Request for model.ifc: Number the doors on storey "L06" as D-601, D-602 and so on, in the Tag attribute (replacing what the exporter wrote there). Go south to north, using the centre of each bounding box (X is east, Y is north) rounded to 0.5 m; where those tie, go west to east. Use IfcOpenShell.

First a look at what the model holds.

```python
import ifcopenshell
import ifcopenshell.util.element
import ifcopenshell.util.placement

model = ifcopenshell.open("model.ifc")
print(model.schema)
storey = next(s for s in model.by_type("IfcBuildingStorey") if s.Name == "L06")
doors = [e for e in ifcopenshell.util.element.get_decomposition(storey) if e.is_a("IfcDoor")]
for e in sorted(doors, key=lambda e: e.id()):
    origin = ifcopenshell.util.placement.get_local_placement(e.ObjectPlacement)[:3, 3]
    print(e.id(), e.Tag, e.Name, origin.round(2) + 0.0, sep=" | ")
```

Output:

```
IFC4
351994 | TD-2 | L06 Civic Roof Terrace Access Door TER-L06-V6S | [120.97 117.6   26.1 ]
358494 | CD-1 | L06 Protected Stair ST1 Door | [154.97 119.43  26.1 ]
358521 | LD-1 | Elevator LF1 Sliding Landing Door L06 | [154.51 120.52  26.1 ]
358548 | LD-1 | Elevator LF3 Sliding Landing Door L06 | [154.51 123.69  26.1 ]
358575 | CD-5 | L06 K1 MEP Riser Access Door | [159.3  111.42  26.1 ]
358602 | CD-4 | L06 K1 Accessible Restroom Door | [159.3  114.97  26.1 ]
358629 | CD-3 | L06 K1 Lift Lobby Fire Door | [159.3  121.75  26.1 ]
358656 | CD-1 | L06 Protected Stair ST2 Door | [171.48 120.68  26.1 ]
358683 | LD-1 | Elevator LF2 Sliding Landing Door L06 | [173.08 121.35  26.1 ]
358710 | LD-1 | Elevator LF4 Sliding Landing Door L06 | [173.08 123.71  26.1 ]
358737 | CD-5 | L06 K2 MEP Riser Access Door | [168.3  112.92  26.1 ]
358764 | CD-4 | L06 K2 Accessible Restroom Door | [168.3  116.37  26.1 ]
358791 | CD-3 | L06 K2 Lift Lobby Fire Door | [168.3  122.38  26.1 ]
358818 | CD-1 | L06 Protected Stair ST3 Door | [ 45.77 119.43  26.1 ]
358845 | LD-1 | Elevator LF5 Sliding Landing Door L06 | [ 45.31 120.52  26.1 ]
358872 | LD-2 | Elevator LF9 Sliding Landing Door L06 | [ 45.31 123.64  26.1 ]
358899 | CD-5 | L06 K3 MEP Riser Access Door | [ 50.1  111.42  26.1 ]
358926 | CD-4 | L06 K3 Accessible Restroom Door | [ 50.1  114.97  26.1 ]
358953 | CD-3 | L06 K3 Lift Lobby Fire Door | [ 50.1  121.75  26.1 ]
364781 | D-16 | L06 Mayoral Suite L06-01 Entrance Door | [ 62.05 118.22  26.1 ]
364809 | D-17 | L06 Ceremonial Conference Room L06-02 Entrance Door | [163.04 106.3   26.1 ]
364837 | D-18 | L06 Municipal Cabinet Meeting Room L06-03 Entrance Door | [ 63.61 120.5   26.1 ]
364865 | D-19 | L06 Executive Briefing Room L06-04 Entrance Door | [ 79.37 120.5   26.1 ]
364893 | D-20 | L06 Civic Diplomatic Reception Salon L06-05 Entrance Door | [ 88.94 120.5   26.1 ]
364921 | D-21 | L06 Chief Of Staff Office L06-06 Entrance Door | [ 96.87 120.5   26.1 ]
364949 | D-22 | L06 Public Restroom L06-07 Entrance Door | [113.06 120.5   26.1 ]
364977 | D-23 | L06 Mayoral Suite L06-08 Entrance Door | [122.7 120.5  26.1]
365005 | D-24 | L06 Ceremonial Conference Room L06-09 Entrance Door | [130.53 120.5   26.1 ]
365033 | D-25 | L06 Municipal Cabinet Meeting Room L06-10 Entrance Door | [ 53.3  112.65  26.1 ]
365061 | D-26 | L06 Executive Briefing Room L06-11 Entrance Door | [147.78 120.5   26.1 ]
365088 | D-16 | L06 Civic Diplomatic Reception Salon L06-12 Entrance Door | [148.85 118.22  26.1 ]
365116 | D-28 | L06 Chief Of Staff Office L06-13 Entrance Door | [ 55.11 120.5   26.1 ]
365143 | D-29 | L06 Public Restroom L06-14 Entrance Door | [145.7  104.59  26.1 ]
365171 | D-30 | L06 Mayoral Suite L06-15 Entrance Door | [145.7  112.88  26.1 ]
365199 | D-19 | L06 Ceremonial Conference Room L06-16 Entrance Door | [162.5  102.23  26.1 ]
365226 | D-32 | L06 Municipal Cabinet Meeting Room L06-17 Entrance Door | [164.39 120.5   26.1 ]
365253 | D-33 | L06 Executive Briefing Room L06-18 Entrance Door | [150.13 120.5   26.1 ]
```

```python
import ifcopenshell
import ifcopenshell.geom
import ifcopenshell.util.element
import ifcopenshell.util.shape

model = ifcopenshell.open("model.ifc")
settings = ifcopenshell.geom.settings()
settings.set("use-world-coords", True)


def centre(element):
    shape = ifcopenshell.geom.create_shape(settings, element)
    return ifcopenshell.util.shape.get_bbox_centroid(shape.geometry)


storey = next(s for s in model.by_type("IfcBuildingStorey") if s.Name == "L06")
doors = [e for e in ifcopenshell.util.element.get_decomposition(storey) if e.is_a("IfcDoor")]

# Insertion points can sit at a corner or the storey origin, so sort by the geometry (in metres).
centres = {e: centre(e) for e in doors}
doors.sort(key=lambda e: (round(centres[e][1] / 0.5), centres[e][0]))

for i, e in enumerate(doors, start=1):
    number = f"D-6{i:02d}"
    e.Tag = number
    print(e.id(), number)

model.write("model_v2.ifc")
```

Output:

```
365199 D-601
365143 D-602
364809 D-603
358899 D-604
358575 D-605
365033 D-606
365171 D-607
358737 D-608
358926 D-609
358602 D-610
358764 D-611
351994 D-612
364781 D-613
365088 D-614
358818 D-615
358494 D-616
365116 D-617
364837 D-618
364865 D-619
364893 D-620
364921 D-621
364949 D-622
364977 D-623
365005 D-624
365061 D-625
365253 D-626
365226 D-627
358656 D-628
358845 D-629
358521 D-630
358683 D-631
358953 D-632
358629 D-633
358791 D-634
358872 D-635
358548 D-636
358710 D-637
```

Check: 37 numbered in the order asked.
